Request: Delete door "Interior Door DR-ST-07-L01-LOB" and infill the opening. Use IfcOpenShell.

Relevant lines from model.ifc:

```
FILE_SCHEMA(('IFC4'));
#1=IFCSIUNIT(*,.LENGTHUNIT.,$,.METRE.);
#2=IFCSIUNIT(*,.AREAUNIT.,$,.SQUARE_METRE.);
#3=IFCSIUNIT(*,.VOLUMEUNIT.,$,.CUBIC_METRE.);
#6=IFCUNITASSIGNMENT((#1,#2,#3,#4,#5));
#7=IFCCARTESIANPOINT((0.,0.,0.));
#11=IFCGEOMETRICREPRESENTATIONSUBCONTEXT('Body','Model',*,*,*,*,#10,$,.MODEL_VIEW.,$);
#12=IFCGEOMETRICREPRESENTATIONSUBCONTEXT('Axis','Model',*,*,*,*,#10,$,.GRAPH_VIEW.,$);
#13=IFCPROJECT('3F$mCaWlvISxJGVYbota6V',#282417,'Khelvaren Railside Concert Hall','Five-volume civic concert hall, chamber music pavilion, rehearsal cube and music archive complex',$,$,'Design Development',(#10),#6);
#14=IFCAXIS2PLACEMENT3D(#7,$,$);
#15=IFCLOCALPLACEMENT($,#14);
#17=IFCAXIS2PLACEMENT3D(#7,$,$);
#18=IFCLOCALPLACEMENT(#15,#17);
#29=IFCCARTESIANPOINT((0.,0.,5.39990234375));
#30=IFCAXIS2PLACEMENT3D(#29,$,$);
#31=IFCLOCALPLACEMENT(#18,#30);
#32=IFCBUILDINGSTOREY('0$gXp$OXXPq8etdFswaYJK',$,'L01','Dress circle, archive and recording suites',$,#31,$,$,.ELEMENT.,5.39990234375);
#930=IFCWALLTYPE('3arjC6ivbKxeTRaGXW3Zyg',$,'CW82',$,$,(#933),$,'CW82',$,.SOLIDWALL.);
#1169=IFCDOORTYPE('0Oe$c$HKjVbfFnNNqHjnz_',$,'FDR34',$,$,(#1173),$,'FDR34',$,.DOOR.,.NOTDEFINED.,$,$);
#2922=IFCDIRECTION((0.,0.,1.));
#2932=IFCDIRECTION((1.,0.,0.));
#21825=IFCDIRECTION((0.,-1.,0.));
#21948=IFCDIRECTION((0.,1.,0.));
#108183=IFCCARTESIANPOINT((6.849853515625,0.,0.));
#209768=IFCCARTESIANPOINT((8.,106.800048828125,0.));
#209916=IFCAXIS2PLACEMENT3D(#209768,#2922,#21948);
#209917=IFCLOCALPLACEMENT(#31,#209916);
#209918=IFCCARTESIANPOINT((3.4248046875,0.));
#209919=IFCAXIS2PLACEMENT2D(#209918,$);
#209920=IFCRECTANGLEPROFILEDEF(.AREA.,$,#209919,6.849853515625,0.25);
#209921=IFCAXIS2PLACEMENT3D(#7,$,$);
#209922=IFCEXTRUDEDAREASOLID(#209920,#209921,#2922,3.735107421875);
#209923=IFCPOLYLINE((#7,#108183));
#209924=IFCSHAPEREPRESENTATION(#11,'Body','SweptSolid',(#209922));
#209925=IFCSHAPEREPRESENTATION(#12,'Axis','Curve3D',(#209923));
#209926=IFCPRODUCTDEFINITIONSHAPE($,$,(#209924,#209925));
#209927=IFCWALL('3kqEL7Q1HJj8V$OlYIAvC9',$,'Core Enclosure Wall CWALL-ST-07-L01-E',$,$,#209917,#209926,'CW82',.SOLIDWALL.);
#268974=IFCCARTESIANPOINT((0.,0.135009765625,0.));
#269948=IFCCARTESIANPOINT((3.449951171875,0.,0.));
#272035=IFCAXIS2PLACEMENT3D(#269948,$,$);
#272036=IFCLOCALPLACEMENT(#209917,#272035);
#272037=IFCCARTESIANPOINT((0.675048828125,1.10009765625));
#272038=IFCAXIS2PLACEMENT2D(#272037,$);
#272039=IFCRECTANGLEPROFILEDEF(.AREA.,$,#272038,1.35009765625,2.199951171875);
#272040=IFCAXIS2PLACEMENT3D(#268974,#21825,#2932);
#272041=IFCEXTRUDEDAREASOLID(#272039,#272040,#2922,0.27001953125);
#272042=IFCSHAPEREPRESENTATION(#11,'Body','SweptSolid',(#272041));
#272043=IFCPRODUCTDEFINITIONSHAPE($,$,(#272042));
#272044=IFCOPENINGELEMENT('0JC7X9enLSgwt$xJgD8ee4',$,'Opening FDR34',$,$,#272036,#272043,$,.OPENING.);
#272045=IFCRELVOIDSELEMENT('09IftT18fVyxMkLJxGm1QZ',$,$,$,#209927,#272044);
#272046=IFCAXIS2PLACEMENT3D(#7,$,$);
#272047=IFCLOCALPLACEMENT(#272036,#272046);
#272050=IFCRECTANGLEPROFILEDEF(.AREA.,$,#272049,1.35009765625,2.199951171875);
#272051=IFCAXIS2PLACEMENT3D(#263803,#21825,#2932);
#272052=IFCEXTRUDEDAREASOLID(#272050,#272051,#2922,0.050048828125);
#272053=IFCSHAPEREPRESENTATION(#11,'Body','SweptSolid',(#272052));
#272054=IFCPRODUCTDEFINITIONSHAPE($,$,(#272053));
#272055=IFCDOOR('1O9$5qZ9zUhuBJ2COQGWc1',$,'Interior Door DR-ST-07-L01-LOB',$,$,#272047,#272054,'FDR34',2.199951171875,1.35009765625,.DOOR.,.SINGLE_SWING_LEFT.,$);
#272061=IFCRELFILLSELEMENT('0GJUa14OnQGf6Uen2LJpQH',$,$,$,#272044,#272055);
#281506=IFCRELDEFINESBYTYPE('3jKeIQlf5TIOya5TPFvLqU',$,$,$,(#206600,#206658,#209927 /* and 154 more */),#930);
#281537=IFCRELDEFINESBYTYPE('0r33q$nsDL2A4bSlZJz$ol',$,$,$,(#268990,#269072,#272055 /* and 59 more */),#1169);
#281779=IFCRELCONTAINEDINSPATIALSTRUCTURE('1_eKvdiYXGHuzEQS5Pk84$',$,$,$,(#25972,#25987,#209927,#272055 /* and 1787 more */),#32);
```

```python
import ifcopenshell
import ifcopenshell.api.feature
import ifcopenshell.api.root
import ifcopenshell.geom
import ifcopenshell.util.shape

model = ifcopenshell.open("model.ifc")
settings = ifcopenshell.geom.settings()


def volume(element):
    """Net volume in cubic metres, openings subtracted."""
    shape = ifcopenshell.geom.create_shape(settings, element)
    return ifcopenshell.util.shape.get_volume(shape.geometry)


door = model.by_guid("1O9$5qZ9zUhuBJ2COQGWc1")
opening = door.FillsVoids[0].RelatingOpeningElement
wall = opening.VoidsElements[0].RelatingBuildingElement
before = volume(wall)

ifcopenshell.api.root.remove_product(model, product=door)
ifcopenshell.api.feature.remove_feature(model, feature=opening)

after = volume(wall)

print(f"wall volume {before:.3f} -> {after:.3f} m3")

model.write("model_rev.ifc")
```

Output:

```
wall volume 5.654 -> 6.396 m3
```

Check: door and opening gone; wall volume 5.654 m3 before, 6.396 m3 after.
